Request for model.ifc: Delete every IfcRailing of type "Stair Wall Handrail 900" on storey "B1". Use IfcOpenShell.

First a look at what the model holds.

```python
import ifcopenshell
import ifcopenshell.util.element

model = ifcopenshell.open("model.ifc")
print(model.schema)
storey = next(s for s in model.by_type("IfcBuildingStorey") if s.Name == "B1")
railings = [e for e in ifcopenshell.util.element.get_decomposition(storey) if e.is_a("IfcRailing")]
seen = {}
for e in railings:
    element_type = ifcopenshell.util.element.get_type(e)
    name = element_type.Name if element_type not in (None, e) else None
    seen[name] = seen.get(name, 0) + 1
for name, count in sorted(seen.items(), key=str):
    print(count, "x", name)
```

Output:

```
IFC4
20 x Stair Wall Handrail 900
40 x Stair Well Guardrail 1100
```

```python
import ifcopenshell
import ifcopenshell.api.root
import ifcopenshell.util.element

model = ifcopenshell.open("model.ifc")

storey = next(s for s in model.by_type("IfcBuildingStorey") if s.Name == "B1")
railings = [e for e in ifcopenshell.util.element.get_decomposition(storey) if e.is_a("IfcRailing")]
targets = [e for e in railings if (t := ifcopenshell.util.element.get_type(e)) not in (None, e) and t.Name == "Stair Wall Handrail 900"]

for e in targets:
    ifcopenshell.api.root.remove_product(model, product=e)
print(len(targets), "removed")

model.write("model_rev.ifc")
```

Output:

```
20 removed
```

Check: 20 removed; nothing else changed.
